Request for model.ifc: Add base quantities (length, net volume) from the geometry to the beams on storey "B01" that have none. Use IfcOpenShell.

First a look at what the model holds.

```python
import ifcopenshell
import ifcopenshell.util.element
import ifcopenshell.util.unit

model = ifcopenshell.open("model.ifc")
print(model.schema)
for unit_type in ("LENGTHUNIT", "AREAUNIT", "VOLUMEUNIT"):
    print(unit_type, ifcopenshell.util.unit.calculate_unit_scale(model, unit_type))
storey = next(s for s in model.by_type("IfcBuildingStorey") if s.Name == "B01")
beams = [e for e in ifcopenshell.util.element.get_decomposition(storey) if e.is_a("IfcBeam")]
for e in sorted(beams, key=lambda e: e.id()):
    print(e.id(), e.is_a(), e.Name, list(ifcopenshell.util.element.get_psets(e, qtos_only=True)), sep=" | ")
```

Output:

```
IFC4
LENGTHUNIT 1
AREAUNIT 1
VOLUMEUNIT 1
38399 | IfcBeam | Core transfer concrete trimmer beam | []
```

```python
import ifcopenshell
import ifcopenshell.api.pset
import ifcopenshell.geom
import ifcopenshell.util.element
import ifcopenshell.util.shape
import ifcopenshell.util.unit

model = ifcopenshell.open("model.ifc")
unit_scale = ifcopenshell.util.unit.calculate_unit_scale(model)
volume_scale = ifcopenshell.util.unit.calculate_unit_scale(model, "VOLUMEUNIT")
settings = ifcopenshell.geom.settings()

storey = next(s for s in model.by_type("IfcBuildingStorey") if s.Name == "B01")
beams = [e for e in ifcopenshell.util.element.get_decomposition(storey) if e.is_a("IfcBeam")]

for e in sorted(beams, key=lambda e: e.id()):
    if ifcopenshell.util.element.get_psets(e, qtos_only=True, should_inherit=False):
        continue
    # Geometry comes back in metres, in the element's own axes.
    shape = ifcopenshell.geom.create_shape(settings, e)
    values = {
        "Length": ifcopenshell.util.shape.get_max_xyz(shape.geometry) / unit_scale,
        "NetVolume": ifcopenshell.util.shape.get_volume(shape.geometry) / volume_scale,
    }
    qto = ifcopenshell.api.pset.add_qto(model, product=e, name="Qto_BeamBaseQuantities")
    ifcopenshell.api.pset.edit_qto(model, qto=qto, properties=values)
    print(e.id(), {k: round(v, 3) for k, v in values.items()})

model.write("model_v2.ifc")
```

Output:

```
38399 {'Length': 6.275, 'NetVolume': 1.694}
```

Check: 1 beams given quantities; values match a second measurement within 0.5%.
